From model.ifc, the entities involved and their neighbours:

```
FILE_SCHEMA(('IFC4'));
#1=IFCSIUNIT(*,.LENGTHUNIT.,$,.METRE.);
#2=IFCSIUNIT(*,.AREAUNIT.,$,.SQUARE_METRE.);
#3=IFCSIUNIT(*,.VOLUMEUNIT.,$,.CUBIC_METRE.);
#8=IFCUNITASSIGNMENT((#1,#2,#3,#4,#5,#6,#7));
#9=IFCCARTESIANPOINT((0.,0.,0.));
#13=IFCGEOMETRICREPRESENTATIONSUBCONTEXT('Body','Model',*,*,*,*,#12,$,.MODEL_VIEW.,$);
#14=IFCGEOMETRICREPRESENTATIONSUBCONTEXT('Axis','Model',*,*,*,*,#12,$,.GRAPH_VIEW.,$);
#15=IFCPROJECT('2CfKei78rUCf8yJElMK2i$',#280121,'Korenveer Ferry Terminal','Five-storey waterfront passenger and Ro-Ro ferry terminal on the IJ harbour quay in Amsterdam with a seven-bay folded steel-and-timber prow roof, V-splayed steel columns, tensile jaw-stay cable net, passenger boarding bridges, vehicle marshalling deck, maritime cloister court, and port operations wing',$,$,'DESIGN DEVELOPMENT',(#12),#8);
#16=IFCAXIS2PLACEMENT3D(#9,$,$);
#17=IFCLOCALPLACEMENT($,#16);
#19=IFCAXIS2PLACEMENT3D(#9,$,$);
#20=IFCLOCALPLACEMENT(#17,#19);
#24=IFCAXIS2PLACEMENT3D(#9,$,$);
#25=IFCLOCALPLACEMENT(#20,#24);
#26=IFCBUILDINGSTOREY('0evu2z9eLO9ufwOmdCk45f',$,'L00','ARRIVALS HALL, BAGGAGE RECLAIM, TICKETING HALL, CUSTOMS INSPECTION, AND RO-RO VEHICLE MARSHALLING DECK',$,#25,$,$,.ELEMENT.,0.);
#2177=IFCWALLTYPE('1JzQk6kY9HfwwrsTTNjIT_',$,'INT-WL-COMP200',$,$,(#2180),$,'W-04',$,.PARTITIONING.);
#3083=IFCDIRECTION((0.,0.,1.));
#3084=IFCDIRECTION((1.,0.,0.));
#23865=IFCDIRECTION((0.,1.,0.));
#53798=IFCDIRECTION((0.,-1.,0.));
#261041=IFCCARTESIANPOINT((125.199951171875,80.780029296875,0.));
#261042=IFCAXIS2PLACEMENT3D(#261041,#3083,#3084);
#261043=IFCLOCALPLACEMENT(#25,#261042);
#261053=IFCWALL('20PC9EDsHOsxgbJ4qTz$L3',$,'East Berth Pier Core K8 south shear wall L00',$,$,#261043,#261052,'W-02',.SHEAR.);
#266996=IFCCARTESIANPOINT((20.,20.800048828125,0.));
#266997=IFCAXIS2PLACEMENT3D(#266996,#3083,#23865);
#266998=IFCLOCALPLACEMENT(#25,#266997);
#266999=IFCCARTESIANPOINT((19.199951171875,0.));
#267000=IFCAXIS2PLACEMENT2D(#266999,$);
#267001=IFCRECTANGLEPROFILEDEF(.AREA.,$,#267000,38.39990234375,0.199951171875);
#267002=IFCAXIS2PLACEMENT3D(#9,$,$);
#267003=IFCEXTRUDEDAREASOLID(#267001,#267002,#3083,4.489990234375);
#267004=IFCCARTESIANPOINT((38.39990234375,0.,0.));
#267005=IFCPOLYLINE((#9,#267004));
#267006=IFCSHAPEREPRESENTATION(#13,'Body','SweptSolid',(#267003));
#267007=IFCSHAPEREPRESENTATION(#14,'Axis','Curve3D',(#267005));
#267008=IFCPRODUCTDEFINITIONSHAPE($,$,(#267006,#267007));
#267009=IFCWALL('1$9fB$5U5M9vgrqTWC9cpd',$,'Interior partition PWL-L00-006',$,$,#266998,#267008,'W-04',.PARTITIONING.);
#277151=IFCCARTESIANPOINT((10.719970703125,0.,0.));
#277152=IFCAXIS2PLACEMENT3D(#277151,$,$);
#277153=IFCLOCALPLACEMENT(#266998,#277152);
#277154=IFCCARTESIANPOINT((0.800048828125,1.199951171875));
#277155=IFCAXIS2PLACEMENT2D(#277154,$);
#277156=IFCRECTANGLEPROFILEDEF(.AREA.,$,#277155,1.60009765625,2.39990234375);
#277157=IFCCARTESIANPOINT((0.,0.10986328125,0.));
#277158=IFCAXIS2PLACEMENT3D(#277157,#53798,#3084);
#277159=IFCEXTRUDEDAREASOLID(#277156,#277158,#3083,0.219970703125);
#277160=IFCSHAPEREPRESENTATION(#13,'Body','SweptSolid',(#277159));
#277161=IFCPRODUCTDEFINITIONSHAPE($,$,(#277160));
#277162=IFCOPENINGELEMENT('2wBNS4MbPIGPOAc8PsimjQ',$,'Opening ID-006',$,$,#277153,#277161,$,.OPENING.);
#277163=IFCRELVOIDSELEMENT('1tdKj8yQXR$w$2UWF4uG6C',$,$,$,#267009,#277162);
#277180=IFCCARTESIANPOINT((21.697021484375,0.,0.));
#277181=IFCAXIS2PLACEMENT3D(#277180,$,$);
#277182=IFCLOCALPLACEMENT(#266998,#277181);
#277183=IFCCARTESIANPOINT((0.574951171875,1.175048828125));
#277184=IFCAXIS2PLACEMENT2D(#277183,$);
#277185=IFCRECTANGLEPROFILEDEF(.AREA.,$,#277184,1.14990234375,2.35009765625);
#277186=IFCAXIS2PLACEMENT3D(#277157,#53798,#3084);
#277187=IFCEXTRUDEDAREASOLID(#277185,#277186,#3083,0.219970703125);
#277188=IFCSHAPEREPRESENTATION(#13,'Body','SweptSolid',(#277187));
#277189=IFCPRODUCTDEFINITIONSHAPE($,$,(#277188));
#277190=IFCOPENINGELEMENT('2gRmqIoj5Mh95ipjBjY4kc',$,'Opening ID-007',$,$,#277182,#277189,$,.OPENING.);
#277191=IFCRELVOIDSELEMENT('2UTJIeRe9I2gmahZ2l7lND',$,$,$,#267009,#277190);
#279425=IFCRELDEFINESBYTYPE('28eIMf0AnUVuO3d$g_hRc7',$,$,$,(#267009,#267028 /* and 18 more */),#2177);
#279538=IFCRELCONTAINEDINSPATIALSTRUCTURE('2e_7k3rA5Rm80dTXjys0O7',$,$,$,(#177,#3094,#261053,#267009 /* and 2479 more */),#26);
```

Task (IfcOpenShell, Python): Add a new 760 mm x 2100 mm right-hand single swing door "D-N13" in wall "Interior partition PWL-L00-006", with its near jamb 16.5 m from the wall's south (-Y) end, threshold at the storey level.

```python
import numpy as np
import ifcopenshell
import ifcopenshell.api.feature
import ifcopenshell.api.geometry
import ifcopenshell.api.root
import ifcopenshell.api.spatial
import ifcopenshell.geom
import ifcopenshell.util.element
import ifcopenshell.util.placement
import ifcopenshell.util.representation
import ifcopenshell.util.shape
import ifcopenshell.util.unit

model = ifcopenshell.open("model.ifc")
unit_scale = ifcopenshell.util.unit.calculate_unit_scale(model)
settings = ifcopenshell.geom.settings()


def volume(element):
    """Net volume in cubic metres, openings subtracted."""
    shape = ifcopenshell.geom.create_shape(settings, element)
    return ifcopenshell.util.shape.get_volume(shape.geometry)


wall = model.by_guid("1$9fB$5U5M9vgrqTWC9cpd")
storey = ifcopenshell.util.element.get_container(wall, ifc_class="IfcBuildingStorey")
context = ifcopenshell.util.representation.get_context(model, "Model", "Body", "MODEL_VIEW")
before = volume(wall)

width, height, from_end, sill = 0.76, 2.1, 16.5, 0.0  # metres

# The wall runs along its own X axis, and the end named is its -X end.
wall_shape = ifcopenshell.geom.create_shape(settings, wall)
x, y, z = ifcopenshell.util.shape.get_vertices(wall_shape.geometry).T
start = x.min() + from_end
face, thickness = float(y.min()), float(y.max() - y.min())
wall_matrix = ifcopenshell.util.placement.get_local_placement(wall.ObjectPlacement)
level = ifcopenshell.util.placement.get_local_placement(storey.ObjectPlacement)[2, 3]


def in_wall(x, y):
    """Placement at x, y metres in the wall's axes, at sill height."""
    matrix = wall_matrix.copy()
    matrix[:, 3] = wall_matrix @ np.array([x / unit_scale, y / unit_scale, 0.0, 1.0])
    matrix[2, 3] = level + sill / unit_scale
    return matrix


# Opening: a box that overshoots both wall faces by 50 mm.
opening = ifcopenshell.api.root.create_entity(model, ifc_class="IfcOpeningElement", predefined_type="OPENING")
box = ifcopenshell.api.geometry.add_wall_representation(
    model, context=context, length=width, height=height, thickness=thickness + 0.1
)
ifcopenshell.api.geometry.assign_representation(model, product=opening, representation=box)
ifcopenshell.api.geometry.edit_object_placement(model, product=opening, matrix=in_wall(start, face - 0.05), is_si=False)
ifcopenshell.api.feature.add_feature(model, feature=opening, element=wall)

door = ifcopenshell.api.root.create_entity(model, ifc_class="IfcDoor", name="D-N13", predefined_type="DOOR")
door.OverallWidth, door.OverallHeight = width / unit_scale, height / unit_scale
door.OperationType = "SINGLE_SWING_RIGHT"
body = ifcopenshell.api.geometry.add_door_representation(
    model,
    context=context,
    overall_width=door.OverallWidth,
    overall_height=door.OverallHeight,
    operation_type="SINGLE_SWING_RIGHT",
    lining_properties={"LiningDepth": thickness / unit_scale, "ThresholdDepth": thickness / unit_scale},
)
ifcopenshell.api.geometry.assign_representation(model, product=door, representation=body)
ifcopenshell.api.spatial.assign_container(model, products=[door], relating_structure=storey)
ifcopenshell.api.feature.add_filling(model, opening=opening, element=door)

# The lining spans the wall, so the door starts at the wall face.
ifcopenshell.api.geometry.edit_object_placement(model, product=door, matrix=in_wall(start, face), is_si=False)

after = volume(wall)

print(f"wall volume {before:.3f} -> {after:.3f} m3")

model.write("model_v2.ifc")
```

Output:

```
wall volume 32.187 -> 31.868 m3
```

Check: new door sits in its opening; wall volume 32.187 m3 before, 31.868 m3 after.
